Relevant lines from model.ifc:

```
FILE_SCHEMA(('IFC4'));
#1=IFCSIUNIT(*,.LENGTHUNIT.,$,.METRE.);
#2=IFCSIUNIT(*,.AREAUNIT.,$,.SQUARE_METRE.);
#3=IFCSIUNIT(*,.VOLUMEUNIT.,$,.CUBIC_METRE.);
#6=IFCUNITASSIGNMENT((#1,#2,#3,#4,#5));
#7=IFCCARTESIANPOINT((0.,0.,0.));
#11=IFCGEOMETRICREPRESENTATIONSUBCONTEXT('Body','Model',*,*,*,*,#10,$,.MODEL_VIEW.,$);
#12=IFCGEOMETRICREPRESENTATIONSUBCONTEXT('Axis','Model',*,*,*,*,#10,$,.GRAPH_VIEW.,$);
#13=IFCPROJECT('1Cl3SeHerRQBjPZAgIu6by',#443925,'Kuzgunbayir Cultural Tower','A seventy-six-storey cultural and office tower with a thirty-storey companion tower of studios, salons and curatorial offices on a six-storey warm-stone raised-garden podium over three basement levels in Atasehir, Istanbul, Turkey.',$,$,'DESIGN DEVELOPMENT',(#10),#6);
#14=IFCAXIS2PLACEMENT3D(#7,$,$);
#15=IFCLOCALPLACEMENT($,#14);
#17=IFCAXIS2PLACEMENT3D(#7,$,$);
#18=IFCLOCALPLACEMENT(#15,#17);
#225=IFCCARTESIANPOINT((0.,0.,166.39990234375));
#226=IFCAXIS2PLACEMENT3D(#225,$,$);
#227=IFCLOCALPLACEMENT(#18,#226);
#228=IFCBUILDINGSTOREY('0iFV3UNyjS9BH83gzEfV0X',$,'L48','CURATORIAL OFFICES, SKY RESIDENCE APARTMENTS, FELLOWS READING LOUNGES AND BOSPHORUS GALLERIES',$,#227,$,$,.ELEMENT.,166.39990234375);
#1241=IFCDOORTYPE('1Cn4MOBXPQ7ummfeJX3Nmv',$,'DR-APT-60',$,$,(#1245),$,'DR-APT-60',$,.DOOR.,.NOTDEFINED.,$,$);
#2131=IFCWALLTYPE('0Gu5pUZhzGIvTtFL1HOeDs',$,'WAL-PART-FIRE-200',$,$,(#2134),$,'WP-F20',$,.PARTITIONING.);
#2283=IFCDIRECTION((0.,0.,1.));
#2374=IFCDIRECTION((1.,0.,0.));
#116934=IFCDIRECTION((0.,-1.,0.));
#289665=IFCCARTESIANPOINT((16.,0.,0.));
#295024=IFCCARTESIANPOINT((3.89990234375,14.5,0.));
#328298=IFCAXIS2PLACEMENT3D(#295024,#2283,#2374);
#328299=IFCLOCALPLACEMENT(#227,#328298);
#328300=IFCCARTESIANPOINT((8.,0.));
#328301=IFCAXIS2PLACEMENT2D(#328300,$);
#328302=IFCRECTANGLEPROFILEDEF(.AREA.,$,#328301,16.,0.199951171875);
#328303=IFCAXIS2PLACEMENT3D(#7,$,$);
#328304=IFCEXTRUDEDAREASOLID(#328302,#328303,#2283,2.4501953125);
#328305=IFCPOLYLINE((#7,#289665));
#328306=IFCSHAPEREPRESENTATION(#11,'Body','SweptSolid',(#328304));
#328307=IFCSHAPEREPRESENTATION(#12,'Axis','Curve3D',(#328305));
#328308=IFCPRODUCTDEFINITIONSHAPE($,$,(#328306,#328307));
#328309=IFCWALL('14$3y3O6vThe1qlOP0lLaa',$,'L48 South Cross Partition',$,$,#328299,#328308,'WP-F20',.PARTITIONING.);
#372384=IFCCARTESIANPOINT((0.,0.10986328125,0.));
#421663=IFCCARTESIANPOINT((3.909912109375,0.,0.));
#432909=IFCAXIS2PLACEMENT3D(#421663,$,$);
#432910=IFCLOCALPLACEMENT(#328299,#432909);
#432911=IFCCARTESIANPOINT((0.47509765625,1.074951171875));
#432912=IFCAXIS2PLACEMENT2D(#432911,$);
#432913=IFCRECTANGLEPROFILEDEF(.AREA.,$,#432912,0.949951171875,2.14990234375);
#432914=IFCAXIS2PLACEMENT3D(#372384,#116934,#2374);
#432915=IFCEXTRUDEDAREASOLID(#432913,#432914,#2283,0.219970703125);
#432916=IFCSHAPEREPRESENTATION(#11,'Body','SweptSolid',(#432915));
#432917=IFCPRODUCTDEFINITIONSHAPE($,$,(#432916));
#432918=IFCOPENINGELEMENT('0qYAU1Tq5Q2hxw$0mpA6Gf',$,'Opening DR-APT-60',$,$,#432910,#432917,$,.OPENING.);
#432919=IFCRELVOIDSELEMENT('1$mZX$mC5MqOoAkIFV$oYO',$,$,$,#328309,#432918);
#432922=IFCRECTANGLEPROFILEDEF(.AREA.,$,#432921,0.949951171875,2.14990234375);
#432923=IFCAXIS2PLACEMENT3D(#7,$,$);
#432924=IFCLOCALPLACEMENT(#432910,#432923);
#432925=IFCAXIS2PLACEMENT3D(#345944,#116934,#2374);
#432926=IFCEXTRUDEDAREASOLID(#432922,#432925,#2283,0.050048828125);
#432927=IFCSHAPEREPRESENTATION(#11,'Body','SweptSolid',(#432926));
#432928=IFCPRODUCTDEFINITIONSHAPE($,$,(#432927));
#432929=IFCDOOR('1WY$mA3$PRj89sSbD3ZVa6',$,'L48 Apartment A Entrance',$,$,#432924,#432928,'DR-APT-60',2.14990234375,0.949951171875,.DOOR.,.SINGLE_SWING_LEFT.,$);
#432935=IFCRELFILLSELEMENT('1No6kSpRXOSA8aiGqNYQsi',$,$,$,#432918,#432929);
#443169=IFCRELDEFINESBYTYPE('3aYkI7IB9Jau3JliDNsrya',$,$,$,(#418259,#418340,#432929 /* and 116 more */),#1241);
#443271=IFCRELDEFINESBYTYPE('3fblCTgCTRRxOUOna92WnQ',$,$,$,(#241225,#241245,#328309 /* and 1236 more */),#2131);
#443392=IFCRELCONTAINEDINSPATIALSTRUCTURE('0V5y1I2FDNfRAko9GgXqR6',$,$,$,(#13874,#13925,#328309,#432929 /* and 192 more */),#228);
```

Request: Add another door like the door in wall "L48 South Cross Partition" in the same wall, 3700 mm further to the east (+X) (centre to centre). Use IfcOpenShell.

```python
import ifcopenshell
import ifcopenshell.api.feature
import ifcopenshell.api.geometry
import ifcopenshell.api.root
import ifcopenshell.geom
import ifcopenshell.util.element
import ifcopenshell.util.placement
import ifcopenshell.util.shape

model = ifcopenshell.open("model.ifc")
settings = ifcopenshell.geom.settings()


def volume(element):
    """Net volume in cubic metres, openings subtracted."""
    shape = ifcopenshell.geom.create_shape(settings, element)
    return ifcopenshell.util.shape.get_volume(shape.geometry)


door = model.by_id(432929)
opening = door.FillsVoids[0].RelatingOpeningElement
wall = opening.VoidsElements[0].RelatingBuildingElement
before = volume(wall)
shift = ifcopenshell.util.placement.get_local_placement(wall.ObjectPlacement)[:3, 0] * 3.7

# copy_class copies the void relationship, type, container and properties, but no geometry.
new_opening = ifcopenshell.api.root.copy_class(model, product=opening)
new_opening.Representation = ifcopenshell.util.element.copy_deep(
    model, opening.Representation, exclude=["IfcGeometricRepresentationContext", "IfcRepresentationMap"]
)
new_door = ifcopenshell.api.root.copy_class(model, product=door)
new_door.Representation = ifcopenshell.util.element.copy_deep(
    model, door.Representation, exclude=["IfcGeometricRepresentationContext", "IfcRepresentationMap"]
)
new_door.Tag = None
ifcopenshell.api.feature.add_filling(model, opening=new_opening, element=new_door)

for old, new in ((opening, new_opening), (door, new_door)):
    matrix = ifcopenshell.util.placement.get_local_placement(old.ObjectPlacement)
    matrix[:3, 3] += shift
    ifcopenshell.api.geometry.edit_object_placement(model, product=new, matrix=matrix, is_si=False)

after = volume(wall)

print(f"wall volume {before:.3f} -> {after:.3f} m3")

model.write("model_updated.ifc")
```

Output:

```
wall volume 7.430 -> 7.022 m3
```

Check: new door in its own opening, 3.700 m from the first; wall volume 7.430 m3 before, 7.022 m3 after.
